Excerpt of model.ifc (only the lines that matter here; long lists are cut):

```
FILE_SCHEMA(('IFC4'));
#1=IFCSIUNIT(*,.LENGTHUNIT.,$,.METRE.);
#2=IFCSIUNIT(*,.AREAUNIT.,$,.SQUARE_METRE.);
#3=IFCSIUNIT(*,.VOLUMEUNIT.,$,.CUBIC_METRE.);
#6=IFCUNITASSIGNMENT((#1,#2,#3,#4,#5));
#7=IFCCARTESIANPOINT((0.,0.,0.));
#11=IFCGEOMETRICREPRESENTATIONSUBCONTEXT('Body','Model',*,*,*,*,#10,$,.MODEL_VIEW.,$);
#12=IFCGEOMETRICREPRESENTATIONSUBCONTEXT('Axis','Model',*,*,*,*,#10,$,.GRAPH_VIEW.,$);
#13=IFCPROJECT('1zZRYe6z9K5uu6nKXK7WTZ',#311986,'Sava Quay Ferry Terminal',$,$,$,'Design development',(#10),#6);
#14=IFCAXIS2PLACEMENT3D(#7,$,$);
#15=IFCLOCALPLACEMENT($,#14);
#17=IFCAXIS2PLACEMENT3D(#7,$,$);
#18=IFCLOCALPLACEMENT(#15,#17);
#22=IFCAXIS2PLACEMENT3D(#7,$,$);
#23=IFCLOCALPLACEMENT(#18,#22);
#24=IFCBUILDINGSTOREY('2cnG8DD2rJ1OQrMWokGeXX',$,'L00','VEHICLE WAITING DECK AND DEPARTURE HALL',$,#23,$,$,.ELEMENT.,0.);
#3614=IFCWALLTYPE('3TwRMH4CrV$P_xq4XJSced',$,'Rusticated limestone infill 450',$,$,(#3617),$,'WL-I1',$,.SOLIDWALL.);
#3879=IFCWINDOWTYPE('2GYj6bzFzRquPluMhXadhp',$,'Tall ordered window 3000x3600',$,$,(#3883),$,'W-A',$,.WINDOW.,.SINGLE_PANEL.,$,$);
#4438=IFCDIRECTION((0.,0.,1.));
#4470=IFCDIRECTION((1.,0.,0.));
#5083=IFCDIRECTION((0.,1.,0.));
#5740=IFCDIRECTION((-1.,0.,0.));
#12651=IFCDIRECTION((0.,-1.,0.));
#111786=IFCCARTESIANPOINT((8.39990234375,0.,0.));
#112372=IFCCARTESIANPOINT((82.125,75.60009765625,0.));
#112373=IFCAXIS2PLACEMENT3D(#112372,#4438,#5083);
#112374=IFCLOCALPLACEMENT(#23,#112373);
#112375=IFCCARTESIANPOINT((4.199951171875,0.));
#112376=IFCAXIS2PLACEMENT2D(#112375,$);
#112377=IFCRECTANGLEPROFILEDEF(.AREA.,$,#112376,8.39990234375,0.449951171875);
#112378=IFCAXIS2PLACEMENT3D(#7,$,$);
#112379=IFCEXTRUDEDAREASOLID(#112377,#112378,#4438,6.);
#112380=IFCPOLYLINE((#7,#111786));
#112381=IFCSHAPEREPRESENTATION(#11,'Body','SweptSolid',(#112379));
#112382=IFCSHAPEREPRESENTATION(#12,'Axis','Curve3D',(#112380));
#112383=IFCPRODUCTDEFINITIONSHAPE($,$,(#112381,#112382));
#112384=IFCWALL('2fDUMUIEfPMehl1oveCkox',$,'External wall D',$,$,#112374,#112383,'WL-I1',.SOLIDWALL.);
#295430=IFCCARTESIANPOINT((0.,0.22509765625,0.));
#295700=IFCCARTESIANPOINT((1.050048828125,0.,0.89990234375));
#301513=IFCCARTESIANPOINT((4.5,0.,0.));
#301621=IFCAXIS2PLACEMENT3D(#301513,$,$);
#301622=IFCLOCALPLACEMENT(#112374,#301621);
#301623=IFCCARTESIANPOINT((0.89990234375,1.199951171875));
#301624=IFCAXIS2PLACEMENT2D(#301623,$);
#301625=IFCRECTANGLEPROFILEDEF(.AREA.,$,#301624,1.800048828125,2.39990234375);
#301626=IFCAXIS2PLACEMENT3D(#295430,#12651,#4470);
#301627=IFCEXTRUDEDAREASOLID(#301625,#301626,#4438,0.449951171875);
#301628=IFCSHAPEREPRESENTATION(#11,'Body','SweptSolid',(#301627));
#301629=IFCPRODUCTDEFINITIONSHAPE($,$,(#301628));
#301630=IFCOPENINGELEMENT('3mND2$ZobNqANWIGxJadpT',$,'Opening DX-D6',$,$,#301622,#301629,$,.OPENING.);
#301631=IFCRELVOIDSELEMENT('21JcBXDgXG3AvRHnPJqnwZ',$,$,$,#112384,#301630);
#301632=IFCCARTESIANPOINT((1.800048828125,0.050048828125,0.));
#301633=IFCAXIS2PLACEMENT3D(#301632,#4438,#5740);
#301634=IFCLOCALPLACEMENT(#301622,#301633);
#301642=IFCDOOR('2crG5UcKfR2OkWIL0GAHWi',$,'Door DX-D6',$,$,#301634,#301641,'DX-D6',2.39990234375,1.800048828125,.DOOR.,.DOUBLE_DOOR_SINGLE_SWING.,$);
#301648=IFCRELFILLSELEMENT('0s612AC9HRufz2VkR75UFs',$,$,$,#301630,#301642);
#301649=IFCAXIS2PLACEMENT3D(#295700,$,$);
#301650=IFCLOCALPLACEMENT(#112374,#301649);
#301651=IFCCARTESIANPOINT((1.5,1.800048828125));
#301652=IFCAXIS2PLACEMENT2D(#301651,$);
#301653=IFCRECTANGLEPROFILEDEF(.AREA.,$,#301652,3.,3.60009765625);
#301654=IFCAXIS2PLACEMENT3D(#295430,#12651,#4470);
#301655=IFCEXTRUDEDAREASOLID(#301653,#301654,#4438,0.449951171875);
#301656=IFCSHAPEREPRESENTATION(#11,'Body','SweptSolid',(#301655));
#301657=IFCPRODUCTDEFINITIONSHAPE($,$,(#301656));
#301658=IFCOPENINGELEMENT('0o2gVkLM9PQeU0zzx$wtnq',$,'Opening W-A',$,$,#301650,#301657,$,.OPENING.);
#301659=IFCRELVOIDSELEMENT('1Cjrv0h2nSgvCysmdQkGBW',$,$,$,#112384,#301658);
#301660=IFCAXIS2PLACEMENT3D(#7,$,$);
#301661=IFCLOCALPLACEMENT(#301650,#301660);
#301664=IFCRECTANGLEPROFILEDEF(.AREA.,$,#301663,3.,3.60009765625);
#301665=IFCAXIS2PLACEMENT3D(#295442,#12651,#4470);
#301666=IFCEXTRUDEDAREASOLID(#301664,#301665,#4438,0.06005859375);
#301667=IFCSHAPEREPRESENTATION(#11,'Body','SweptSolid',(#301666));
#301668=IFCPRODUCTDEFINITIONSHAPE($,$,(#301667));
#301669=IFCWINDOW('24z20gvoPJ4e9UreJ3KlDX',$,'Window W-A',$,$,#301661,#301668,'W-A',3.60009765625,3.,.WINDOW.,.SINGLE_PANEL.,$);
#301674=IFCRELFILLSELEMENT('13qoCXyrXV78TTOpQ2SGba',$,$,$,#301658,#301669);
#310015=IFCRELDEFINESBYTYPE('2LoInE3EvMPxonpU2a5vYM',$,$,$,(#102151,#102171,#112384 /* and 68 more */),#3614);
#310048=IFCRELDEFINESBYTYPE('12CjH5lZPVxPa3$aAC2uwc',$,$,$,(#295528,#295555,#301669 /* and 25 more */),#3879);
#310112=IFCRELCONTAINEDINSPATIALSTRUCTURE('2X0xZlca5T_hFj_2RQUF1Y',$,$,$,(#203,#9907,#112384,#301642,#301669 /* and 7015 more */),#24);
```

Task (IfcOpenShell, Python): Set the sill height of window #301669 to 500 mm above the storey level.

```python
import numpy as np
import ifcopenshell
import ifcopenshell.api.geometry
import ifcopenshell.geom
import ifcopenshell.util.element
import ifcopenshell.util.placement
import ifcopenshell.util.shape
import ifcopenshell.util.unit

model = ifcopenshell.open("model.ifc")
unit_scale = ifcopenshell.util.unit.calculate_unit_scale(model)

window = model.by_id(301669)
opening = window.FillsVoids[0].RelatingOpeningElement
storey = ifcopenshell.util.element.get_container(window, ifc_class="IfcBuildingStorey")
level = ifcopenshell.util.placement.get_local_placement(storey.ObjectPlacement)[2, 3]

# The opening's origin need not be at the sill, so measure its lowest point.
shape = ifcopenshell.geom.create_shape(ifcopenshell.geom.settings(), opening)
bottom = ifcopenshell.util.shape.get_shape_bottom_elevation(shape, shape.geometry) / unit_scale
dz = level + 0.5 / unit_scale - bottom

shift = np.array([0.0, 0.0, dz])
# The window is placed relative to its opening, so it follows when the opening moves.
matrix = ifcopenshell.util.placement.get_local_placement(opening.ObjectPlacement)
matrix[:3, 3] += shift
ifcopenshell.api.geometry.edit_object_placement(
    model, product=opening, matrix=matrix, is_si=False, should_transform_children=True
)

print(f"moved by {dz * unit_scale:+.3f} m")

model.write("model_v2.ifc")
```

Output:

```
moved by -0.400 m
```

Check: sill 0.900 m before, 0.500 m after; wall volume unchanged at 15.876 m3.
